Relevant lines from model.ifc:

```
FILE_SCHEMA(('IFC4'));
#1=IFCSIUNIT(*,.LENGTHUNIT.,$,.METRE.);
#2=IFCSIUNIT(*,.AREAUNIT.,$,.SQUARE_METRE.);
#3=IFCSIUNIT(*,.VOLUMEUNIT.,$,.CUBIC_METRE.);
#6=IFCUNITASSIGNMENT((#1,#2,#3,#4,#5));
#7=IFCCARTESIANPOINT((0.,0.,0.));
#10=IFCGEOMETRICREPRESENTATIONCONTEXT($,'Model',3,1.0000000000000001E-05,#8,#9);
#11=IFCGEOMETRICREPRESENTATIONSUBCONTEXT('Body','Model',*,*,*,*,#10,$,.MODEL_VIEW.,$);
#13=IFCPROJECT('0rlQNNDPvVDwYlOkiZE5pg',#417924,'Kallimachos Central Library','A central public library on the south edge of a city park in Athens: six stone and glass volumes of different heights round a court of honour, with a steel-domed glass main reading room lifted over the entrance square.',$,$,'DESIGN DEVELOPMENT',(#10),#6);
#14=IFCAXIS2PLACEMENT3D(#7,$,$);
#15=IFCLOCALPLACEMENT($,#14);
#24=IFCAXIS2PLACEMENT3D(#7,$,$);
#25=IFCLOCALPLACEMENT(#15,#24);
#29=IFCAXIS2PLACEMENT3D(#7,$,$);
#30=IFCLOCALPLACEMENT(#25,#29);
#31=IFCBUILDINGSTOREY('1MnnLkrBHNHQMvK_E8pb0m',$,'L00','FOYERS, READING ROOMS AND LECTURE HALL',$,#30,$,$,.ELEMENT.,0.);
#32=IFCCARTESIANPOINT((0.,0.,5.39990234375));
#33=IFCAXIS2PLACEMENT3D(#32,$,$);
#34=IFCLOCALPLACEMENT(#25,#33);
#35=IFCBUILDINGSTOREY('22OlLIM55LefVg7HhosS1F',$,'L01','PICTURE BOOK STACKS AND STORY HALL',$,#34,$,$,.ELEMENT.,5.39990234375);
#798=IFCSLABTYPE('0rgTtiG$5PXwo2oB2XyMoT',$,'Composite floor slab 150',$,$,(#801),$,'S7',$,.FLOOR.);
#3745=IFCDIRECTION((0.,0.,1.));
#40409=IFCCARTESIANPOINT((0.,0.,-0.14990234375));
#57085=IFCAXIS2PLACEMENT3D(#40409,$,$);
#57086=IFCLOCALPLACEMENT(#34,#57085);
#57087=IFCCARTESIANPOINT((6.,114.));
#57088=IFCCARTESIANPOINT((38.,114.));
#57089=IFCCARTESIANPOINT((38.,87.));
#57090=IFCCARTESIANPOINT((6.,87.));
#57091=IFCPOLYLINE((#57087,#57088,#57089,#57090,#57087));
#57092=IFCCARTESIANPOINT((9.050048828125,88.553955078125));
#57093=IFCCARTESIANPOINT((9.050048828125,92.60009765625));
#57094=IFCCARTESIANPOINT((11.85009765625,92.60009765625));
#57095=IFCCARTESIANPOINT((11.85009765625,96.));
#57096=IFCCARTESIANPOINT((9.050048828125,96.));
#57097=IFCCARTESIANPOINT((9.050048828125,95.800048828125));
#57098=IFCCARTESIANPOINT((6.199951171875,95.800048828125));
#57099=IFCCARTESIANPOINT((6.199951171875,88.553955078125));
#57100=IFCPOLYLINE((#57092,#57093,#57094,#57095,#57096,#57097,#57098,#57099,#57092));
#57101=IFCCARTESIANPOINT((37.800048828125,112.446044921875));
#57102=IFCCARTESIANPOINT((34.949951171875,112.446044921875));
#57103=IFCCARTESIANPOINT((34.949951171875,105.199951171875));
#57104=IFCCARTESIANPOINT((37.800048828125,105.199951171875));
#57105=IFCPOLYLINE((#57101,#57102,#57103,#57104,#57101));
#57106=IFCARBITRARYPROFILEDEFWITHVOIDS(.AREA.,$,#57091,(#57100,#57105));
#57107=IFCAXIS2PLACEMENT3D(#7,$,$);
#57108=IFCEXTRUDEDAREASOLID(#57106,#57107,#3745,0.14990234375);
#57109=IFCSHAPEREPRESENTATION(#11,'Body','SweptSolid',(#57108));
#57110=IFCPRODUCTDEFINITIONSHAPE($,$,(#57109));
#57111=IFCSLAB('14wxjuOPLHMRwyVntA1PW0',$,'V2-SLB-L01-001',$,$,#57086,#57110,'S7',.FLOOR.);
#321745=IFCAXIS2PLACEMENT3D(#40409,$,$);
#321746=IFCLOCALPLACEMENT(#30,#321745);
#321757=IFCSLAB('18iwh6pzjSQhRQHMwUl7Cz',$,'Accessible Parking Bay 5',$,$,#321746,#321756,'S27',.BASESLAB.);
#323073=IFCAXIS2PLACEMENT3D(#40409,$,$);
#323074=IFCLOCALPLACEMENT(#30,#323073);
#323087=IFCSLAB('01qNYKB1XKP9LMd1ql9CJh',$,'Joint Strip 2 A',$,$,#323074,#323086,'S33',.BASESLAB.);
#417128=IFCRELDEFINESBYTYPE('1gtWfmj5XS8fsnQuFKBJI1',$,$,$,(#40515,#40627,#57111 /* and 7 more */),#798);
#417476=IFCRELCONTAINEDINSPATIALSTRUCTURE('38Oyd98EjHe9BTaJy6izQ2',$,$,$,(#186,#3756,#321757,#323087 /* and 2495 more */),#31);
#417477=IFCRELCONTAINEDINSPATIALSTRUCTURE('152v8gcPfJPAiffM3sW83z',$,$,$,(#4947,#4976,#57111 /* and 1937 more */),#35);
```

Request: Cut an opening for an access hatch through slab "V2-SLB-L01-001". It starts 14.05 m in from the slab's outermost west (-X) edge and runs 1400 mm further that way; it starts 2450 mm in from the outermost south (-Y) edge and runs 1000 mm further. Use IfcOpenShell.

```python
import numpy as np
import ifcopenshell
import ifcopenshell.api.feature
import ifcopenshell.api.geometry
import ifcopenshell.api.root
import ifcopenshell.geom
import ifcopenshell.util.placement
import ifcopenshell.util.representation
import ifcopenshell.util.shape
import ifcopenshell.util.unit

model = ifcopenshell.open("model.ifc")
unit_scale = ifcopenshell.util.unit.calculate_unit_scale(model)
settings = ifcopenshell.geom.settings()


def volume(element):
    """Net volume in cubic metres, openings subtracted."""
    shape = ifcopenshell.geom.create_shape(settings, element)
    return ifcopenshell.util.shape.get_volume(shape.geometry)


slab = model.by_id(57111)
before = volume(slab)

# Extent in the slab's own axes, in metres. The edges named are its -X and -Y sides.
slab_shape = ifcopenshell.geom.create_shape(settings, slab)
vertices = ifcopenshell.util.shape.get_vertices(slab_shape.geometry)
x_min, y_min, bottom = vertices.min(axis=0)
top = vertices[:, 2].max()

opening = ifcopenshell.api.root.create_entity(model, ifc_class="IfcOpeningElement", name="Access hatch opening", predefined_type="OPENING")
context = ifcopenshell.util.representation.get_context(model, "Model", "Body", "MODEL_VIEW")
width, depth = 1.4, 1
outline = [(0.0, 0.0), (width, 0.0), (width, depth), (0.0, depth), (0.0, 0.0)]
# Overshoot both faces by 50 mm so the cut is clean.
shape = ifcopenshell.api.geometry.add_slab_representation(
    model, context=context, depth=top - bottom + 0.1, polyline=outline
)
ifcopenshell.api.geometry.assign_representation(model, product=opening, representation=shape)

matrix = ifcopenshell.util.placement.get_local_placement(slab.ObjectPlacement)
matrix[:, 3] = matrix @ np.append(np.array([x_min + 14.05, y_min + 2.45, bottom - 0.05]) / unit_scale, 1.0)
ifcopenshell.api.geometry.edit_object_placement(model, product=opening, matrix=matrix, is_si=False)
ifcopenshell.api.feature.add_feature(model, feature=opening, element=slab)

after = volume(slab)

print(f"slab volume {before:.3f} -> {after:.3f} m3")

model.write("model_v2.ifc")
```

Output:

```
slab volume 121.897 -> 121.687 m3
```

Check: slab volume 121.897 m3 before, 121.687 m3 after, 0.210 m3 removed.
